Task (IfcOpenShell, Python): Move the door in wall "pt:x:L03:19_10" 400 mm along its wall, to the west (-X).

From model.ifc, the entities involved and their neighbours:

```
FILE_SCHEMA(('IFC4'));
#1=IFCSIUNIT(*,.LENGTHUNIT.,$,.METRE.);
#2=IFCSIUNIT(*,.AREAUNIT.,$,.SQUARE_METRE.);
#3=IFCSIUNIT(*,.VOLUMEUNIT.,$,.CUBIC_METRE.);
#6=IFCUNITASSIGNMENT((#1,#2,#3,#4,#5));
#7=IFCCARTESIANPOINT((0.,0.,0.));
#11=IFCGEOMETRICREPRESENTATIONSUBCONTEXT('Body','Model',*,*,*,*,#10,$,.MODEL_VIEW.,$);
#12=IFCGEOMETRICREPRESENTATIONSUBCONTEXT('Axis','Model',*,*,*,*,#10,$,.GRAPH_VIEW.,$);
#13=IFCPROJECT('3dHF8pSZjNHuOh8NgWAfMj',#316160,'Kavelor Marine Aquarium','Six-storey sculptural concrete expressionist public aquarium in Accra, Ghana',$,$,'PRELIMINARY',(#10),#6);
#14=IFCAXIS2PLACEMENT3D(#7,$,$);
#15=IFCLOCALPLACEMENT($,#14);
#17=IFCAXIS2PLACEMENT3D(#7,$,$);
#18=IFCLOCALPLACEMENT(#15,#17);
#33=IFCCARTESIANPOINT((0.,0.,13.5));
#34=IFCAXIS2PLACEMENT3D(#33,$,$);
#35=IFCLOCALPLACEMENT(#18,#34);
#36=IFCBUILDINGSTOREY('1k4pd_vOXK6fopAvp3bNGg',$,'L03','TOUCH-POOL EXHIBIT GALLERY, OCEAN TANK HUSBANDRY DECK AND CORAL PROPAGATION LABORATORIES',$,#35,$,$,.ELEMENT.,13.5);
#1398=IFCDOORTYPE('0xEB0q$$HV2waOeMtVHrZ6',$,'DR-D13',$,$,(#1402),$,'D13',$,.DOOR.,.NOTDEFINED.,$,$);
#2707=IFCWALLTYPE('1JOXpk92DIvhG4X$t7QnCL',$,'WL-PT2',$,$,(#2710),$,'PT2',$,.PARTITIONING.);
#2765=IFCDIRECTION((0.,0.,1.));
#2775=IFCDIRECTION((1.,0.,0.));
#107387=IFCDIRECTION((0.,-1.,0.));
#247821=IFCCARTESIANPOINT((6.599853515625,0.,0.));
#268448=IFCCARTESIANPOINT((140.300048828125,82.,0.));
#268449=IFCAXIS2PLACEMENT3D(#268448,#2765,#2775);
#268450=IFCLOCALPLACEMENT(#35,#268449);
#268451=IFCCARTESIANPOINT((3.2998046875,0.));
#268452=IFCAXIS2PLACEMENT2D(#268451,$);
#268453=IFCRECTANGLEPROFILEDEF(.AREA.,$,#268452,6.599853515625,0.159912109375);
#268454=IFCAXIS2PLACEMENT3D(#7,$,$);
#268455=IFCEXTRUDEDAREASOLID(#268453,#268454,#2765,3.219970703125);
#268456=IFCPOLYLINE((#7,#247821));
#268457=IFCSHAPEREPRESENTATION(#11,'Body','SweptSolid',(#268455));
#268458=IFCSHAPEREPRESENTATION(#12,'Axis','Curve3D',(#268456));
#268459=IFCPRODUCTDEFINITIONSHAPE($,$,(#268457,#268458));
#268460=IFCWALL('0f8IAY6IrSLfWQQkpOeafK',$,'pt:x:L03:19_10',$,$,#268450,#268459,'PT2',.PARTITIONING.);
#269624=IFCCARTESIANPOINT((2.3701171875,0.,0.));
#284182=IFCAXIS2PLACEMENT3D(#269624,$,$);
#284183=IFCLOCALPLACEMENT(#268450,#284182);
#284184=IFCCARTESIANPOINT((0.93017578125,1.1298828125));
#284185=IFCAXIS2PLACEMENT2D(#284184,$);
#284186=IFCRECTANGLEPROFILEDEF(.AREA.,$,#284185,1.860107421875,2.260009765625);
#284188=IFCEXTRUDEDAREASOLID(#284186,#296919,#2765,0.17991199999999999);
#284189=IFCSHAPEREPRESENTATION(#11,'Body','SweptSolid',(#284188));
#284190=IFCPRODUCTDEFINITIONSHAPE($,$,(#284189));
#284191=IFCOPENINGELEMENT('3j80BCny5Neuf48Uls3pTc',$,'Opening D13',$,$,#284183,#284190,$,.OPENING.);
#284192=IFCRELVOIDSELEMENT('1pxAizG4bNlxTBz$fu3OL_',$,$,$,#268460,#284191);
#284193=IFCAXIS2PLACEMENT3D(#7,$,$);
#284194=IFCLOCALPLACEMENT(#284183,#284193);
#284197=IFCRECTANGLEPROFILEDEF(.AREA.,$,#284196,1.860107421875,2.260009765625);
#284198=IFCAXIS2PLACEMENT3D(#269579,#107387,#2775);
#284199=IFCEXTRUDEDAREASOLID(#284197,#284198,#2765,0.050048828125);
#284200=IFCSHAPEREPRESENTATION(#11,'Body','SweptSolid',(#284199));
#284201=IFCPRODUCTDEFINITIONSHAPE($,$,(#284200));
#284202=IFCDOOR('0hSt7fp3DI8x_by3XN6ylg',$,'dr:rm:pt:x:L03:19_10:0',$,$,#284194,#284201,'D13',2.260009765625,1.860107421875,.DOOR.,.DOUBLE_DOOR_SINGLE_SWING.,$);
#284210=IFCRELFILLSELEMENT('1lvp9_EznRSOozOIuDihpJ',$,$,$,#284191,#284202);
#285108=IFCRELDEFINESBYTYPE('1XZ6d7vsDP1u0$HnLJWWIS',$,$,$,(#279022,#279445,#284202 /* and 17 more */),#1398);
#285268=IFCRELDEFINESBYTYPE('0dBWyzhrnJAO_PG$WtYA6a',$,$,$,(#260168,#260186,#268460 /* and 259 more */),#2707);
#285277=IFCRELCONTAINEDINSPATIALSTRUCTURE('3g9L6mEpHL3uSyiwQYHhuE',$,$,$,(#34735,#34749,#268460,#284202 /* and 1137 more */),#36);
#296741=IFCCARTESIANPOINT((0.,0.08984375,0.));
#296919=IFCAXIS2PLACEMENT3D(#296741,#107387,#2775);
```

```python
import ifcopenshell
import ifcopenshell.api.geometry
import ifcopenshell.util.placement
import ifcopenshell.util.unit

model = ifcopenshell.open("model.ifc")
unit_scale = ifcopenshell.util.unit.calculate_unit_scale(model)

door = model.by_guid("0hSt7fp3DI8x_by3XN6ylg")
opening = door.FillsVoids[0].RelatingOpeningElement
wall = opening.VoidsElements[0].RelatingBuildingElement

wall_matrix = ifcopenshell.util.placement.get_local_placement(wall.ObjectPlacement)
shift = wall_matrix[:3, 0] * -0.4 / unit_scale
before = ifcopenshell.util.placement.get_local_placement(door.ObjectPlacement)[:3, 3].copy()

# The door is placed relative to its opening, so it follows when the opening moves.
matrix = ifcopenshell.util.placement.get_local_placement(opening.ObjectPlacement)
matrix[:3, 3] += shift
ifcopenshell.api.geometry.edit_object_placement(
    model, product=opening, matrix=matrix, is_si=False, should_transform_children=True
)

after = ifcopenshell.util.placement.get_local_placement(door.ObjectPlacement)[:3, 3]
print("door moved by", (after - before).round(3) + 0.0)

model.write("model_v2.ifc")
```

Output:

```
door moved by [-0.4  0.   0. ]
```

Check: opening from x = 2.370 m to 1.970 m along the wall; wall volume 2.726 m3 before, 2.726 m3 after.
